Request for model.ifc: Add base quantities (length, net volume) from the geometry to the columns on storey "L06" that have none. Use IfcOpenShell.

First a look at what the model holds.

```python
import ifcopenshell
import ifcopenshell.util.element
import ifcopenshell.util.unit

model = ifcopenshell.open("model.ifc")
print(model.schema)
for unit_type in ("LENGTHUNIT", "AREAUNIT", "VOLUMEUNIT"):
    print(unit_type, ifcopenshell.util.unit.calculate_unit_scale(model, unit_type))
storey = next(s for s in model.by_type("IfcBuildingStorey") if s.Name == "L06")
columns = [e for e in ifcopenshell.util.element.get_decomposition(storey) if e.is_a("IfcColumn")]
for e in sorted(columns, key=lambda e: e.id()):
    print(e.id(), e.is_a(), e.Name, list(ifcopenshell.util.element.get_psets(e, qtos_only=True)), sep=" | ")
```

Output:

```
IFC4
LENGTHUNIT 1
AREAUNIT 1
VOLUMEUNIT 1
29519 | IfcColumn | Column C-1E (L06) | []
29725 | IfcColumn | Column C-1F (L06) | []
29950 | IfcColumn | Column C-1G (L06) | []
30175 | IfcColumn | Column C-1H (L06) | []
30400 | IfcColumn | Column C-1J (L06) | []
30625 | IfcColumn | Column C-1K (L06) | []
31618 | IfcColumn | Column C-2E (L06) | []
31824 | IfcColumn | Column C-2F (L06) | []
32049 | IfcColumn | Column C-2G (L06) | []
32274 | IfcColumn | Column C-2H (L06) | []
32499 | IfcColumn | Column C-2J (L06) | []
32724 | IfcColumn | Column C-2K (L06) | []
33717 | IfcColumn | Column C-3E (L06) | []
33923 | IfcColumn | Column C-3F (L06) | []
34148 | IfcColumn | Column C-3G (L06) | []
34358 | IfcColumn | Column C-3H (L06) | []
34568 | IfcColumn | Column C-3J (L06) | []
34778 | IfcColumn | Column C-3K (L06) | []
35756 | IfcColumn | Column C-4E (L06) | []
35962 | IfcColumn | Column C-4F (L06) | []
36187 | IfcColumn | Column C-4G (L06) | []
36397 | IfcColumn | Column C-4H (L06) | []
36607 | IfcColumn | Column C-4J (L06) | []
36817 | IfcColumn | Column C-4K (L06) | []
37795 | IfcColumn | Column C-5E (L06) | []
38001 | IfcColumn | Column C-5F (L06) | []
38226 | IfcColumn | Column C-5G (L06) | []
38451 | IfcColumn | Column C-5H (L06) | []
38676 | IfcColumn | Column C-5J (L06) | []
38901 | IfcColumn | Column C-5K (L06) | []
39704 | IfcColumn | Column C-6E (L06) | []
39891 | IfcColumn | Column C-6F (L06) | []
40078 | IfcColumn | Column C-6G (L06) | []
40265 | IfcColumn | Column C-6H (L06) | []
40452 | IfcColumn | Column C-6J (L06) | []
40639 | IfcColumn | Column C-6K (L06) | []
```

```python
import ifcopenshell
import ifcopenshell.api.pset
import ifcopenshell.geom
import ifcopenshell.util.element
import ifcopenshell.util.shape
import ifcopenshell.util.unit

model = ifcopenshell.open("model.ifc")
unit_scale = ifcopenshell.util.unit.calculate_unit_scale(model)
volume_scale = ifcopenshell.util.unit.calculate_unit_scale(model, "VOLUMEUNIT")
settings = ifcopenshell.geom.settings()

storey = next(s for s in model.by_type("IfcBuildingStorey") if s.Name == "L06")
columns = [e for e in ifcopenshell.util.element.get_decomposition(storey) if e.is_a("IfcColumn")]

for e in sorted(columns, key=lambda e: e.id()):
    if ifcopenshell.util.element.get_psets(e, qtos_only=True, should_inherit=False):
        continue
    # Geometry comes back in metres, in the element's own axes.
    shape = ifcopenshell.geom.create_shape(settings, e)
    values = {
        "Length": ifcopenshell.util.shape.get_z(shape.geometry) / unit_scale,
        "NetVolume": ifcopenshell.util.shape.get_volume(shape.geometry) / volume_scale,
    }
    qto = ifcopenshell.api.pset.add_qto(model, product=e, name="Qto_ColumnBaseQuantities")
    ifcopenshell.api.pset.edit_qto(model, qto=qto, properties=values)
    print(e.id(), {k: round(v, 3) for k, v in values.items()})

model.write("model_v2.ifc")
```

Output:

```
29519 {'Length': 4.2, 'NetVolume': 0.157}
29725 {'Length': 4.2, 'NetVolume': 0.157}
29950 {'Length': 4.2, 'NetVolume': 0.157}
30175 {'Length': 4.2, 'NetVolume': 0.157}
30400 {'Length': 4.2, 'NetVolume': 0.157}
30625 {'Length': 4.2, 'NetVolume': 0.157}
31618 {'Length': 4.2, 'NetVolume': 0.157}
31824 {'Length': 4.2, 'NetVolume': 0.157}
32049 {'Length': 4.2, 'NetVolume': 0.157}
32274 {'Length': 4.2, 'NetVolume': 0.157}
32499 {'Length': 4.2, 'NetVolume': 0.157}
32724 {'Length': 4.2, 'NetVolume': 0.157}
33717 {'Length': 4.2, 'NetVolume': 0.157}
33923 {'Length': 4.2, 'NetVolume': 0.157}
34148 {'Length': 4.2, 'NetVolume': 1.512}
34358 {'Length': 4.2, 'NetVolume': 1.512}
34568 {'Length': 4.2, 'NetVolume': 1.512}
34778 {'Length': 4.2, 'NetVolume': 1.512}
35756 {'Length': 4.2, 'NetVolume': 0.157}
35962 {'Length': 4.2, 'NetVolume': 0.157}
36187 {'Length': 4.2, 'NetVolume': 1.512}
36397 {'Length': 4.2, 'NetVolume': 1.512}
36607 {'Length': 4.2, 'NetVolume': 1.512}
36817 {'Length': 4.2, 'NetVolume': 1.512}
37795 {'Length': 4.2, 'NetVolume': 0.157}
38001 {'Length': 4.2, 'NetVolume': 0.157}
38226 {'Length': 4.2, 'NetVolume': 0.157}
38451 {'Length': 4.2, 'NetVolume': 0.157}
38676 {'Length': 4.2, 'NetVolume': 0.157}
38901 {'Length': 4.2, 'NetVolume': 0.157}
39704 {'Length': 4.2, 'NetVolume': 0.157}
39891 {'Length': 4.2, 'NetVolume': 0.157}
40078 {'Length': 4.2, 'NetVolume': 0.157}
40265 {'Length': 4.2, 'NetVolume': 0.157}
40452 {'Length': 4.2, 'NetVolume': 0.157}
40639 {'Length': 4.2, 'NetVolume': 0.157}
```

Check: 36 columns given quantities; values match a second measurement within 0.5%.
